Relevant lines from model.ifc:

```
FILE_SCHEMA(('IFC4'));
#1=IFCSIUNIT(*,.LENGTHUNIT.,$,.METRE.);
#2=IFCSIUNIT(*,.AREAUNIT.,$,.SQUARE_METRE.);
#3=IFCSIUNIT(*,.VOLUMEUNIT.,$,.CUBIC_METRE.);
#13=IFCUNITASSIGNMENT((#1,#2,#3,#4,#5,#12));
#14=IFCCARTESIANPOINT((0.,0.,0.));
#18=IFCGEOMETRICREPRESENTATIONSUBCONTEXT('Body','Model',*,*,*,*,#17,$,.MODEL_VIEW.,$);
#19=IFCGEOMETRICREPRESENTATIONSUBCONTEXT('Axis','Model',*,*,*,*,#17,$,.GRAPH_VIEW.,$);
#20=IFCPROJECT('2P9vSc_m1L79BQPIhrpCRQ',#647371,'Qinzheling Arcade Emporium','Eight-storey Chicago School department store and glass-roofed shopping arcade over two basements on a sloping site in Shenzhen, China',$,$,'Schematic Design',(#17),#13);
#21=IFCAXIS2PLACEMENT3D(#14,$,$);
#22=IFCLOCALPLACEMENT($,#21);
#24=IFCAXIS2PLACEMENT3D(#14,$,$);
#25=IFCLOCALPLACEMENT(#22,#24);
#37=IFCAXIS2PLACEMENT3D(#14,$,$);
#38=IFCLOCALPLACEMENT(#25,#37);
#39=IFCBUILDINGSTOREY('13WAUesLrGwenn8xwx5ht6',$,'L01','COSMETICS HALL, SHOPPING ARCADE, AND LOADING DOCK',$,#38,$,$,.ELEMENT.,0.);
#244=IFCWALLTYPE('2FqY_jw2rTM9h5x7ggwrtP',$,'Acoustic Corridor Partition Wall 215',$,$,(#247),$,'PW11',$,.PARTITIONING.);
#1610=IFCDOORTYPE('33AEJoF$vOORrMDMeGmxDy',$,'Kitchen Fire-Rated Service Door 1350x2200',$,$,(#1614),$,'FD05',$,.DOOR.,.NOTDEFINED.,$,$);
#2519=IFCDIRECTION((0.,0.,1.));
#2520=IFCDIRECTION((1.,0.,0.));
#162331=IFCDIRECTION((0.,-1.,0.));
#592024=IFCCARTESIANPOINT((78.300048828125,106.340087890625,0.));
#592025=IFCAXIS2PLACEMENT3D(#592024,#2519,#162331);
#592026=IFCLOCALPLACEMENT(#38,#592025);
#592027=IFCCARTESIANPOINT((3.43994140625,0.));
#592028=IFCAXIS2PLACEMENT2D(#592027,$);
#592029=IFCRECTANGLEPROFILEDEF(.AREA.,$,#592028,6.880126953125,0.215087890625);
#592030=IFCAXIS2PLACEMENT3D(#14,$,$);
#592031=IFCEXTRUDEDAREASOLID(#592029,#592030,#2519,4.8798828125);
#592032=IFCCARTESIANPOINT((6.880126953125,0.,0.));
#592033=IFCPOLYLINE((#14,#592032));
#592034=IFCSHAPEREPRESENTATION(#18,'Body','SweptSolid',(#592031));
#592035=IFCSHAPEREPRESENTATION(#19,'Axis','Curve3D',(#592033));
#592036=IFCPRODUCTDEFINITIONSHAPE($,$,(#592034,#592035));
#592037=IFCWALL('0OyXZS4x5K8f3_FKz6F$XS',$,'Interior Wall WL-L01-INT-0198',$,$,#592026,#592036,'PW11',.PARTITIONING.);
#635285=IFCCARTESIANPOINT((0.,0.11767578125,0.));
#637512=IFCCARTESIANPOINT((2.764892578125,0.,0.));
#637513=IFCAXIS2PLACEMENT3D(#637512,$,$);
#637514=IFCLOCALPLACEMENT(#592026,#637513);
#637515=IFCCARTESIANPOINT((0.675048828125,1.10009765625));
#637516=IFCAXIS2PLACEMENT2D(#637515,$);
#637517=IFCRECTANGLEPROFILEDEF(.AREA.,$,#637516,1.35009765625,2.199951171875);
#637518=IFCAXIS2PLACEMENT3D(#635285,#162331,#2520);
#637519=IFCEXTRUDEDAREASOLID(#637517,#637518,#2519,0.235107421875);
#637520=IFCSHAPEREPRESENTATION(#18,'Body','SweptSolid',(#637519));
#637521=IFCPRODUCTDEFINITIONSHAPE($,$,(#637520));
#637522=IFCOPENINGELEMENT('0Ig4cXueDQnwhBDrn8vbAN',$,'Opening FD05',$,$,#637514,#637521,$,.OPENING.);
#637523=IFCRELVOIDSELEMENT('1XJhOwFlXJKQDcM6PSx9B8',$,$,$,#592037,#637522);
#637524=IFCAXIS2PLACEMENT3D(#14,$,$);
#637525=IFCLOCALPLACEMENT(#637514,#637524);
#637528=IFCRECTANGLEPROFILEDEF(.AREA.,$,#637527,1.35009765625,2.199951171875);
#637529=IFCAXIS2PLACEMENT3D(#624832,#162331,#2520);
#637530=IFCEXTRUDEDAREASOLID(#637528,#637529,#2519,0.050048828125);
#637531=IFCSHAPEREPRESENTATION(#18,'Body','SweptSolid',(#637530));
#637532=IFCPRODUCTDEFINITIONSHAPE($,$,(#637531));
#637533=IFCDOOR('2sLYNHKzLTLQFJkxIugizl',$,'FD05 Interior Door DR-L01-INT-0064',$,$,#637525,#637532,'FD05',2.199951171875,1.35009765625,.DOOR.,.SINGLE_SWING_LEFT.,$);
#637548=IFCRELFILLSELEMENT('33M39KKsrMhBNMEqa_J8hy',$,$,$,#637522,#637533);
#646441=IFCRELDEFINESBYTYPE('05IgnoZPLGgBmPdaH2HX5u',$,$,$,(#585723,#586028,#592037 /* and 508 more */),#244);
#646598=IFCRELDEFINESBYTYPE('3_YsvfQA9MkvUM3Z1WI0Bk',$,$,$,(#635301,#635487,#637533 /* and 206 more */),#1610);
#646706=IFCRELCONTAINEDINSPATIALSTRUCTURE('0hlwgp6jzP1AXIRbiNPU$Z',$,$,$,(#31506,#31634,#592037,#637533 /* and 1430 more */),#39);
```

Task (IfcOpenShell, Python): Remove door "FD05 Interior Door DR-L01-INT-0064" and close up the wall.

```python
import ifcopenshell
import ifcopenshell.api.feature
import ifcopenshell.api.root
import ifcopenshell.geom
import ifcopenshell.util.shape

model = ifcopenshell.open("model.ifc")
settings = ifcopenshell.geom.settings()


def volume(element):
    """Net volume in cubic metres, openings subtracted."""
    shape = ifcopenshell.geom.create_shape(settings, element)
    return ifcopenshell.util.shape.get_volume(shape.geometry)


door = model.by_guid("2sLYNHKzLTLQFJkxIugizl")
opening = door.FillsVoids[0].RelatingOpeningElement
wall = opening.VoidsElements[0].RelatingBuildingElement
before = volume(wall)

ifcopenshell.api.root.remove_product(model, product=door)
ifcopenshell.api.feature.remove_feature(model, feature=opening)

after = volume(wall)

print(f"wall volume {before:.3f} -> {after:.3f} m3")

model.write("model_edited.ifc")
```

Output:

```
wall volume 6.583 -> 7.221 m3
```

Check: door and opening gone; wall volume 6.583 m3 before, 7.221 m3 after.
